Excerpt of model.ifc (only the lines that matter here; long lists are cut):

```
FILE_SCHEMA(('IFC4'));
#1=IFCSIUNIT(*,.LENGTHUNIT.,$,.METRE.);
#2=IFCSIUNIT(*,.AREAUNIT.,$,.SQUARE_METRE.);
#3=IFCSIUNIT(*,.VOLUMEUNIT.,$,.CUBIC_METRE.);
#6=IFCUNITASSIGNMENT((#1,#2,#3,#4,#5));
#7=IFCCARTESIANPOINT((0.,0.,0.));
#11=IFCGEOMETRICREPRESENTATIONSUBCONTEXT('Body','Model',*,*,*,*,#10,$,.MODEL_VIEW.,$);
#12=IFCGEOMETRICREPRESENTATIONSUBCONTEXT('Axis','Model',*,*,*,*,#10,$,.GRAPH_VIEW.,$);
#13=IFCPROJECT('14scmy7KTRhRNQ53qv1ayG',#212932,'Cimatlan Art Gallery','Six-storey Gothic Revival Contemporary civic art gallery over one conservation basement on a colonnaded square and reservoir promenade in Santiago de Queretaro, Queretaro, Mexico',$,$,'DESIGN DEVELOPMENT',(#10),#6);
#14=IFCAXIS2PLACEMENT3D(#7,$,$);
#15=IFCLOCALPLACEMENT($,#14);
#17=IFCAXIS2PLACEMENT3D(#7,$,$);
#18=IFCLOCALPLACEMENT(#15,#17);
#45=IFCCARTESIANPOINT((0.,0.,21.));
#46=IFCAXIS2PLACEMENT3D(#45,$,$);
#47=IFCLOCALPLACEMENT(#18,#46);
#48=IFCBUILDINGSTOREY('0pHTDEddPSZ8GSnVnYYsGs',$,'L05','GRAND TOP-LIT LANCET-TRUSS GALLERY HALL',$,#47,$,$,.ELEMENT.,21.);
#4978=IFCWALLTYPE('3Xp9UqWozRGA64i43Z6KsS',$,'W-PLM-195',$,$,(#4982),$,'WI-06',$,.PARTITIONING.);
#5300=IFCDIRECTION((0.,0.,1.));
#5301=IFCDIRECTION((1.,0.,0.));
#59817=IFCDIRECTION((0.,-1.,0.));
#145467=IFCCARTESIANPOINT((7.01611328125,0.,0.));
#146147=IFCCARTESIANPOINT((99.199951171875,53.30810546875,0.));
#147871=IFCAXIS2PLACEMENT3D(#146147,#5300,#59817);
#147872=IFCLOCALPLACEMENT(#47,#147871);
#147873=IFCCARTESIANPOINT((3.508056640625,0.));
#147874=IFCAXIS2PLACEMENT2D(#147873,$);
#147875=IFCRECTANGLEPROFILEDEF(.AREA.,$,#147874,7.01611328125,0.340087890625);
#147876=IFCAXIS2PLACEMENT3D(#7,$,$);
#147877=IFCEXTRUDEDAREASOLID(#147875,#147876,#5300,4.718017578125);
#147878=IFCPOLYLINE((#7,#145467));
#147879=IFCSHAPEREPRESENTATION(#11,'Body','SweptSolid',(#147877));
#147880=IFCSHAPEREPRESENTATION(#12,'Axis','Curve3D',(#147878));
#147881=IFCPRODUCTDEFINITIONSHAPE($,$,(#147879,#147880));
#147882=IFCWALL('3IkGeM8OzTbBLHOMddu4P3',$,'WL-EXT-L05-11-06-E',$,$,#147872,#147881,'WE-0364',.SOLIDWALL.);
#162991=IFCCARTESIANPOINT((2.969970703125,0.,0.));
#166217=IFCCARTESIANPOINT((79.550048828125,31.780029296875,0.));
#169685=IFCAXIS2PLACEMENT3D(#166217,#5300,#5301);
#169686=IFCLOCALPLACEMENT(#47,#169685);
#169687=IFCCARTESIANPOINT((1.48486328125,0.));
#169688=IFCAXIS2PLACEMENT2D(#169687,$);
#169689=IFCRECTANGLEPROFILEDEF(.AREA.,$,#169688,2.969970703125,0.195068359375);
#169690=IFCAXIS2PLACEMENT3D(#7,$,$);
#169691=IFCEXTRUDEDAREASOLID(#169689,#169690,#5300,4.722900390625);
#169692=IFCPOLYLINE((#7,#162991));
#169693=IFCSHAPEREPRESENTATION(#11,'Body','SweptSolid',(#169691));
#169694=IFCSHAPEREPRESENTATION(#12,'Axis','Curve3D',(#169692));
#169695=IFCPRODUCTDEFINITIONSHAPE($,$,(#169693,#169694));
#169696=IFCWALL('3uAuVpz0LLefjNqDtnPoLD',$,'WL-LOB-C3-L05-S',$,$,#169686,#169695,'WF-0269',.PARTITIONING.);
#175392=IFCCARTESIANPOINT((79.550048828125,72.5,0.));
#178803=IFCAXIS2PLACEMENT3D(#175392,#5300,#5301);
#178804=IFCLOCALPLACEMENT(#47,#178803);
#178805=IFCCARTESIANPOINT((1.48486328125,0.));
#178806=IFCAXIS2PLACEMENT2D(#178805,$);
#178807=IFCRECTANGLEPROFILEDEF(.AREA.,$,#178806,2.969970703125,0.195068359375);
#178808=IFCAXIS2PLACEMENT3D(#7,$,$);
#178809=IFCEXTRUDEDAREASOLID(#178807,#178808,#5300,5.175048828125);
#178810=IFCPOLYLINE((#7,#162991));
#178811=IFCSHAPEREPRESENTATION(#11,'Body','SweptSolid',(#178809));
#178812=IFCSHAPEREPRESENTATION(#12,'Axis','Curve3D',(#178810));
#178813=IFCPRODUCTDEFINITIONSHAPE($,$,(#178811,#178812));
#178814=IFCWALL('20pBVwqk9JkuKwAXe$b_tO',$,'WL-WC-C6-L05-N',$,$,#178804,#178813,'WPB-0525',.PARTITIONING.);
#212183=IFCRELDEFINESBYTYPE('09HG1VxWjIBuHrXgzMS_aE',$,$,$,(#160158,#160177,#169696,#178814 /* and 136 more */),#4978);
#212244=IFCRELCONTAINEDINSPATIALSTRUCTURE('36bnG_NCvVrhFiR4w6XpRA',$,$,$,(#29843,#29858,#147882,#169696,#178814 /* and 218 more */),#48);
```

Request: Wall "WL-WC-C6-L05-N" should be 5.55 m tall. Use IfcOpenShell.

```python
import ifcopenshell
import ifcopenshell.geom
import ifcopenshell.util.representation
import ifcopenshell.util.shape

model = ifcopenshell.open("model.ifc")
settings = ifcopenshell.geom.settings()


def volume(element):
    """Net volume in cubic metres, openings subtracted."""
    shape = ifcopenshell.geom.create_shape(settings, element)
    return ifcopenshell.util.shape.get_volume(shape.geometry)


wall = model.by_id(178814)
before = volume(wall)

body = ifcopenshell.util.representation.get_representation(wall, "Model", "Body")
solid = body.Items[0]
old_height = solid.Depth
solid.Depth = 5.55
after = volume(wall)

print(f"height {old_height:g} -> {solid.Depth:g}, volume {before:.3f} -> {after:.3f} m3")

model.write("model_updated.ifc")
```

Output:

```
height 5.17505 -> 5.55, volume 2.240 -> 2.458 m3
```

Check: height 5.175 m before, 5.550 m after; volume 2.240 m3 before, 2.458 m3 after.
